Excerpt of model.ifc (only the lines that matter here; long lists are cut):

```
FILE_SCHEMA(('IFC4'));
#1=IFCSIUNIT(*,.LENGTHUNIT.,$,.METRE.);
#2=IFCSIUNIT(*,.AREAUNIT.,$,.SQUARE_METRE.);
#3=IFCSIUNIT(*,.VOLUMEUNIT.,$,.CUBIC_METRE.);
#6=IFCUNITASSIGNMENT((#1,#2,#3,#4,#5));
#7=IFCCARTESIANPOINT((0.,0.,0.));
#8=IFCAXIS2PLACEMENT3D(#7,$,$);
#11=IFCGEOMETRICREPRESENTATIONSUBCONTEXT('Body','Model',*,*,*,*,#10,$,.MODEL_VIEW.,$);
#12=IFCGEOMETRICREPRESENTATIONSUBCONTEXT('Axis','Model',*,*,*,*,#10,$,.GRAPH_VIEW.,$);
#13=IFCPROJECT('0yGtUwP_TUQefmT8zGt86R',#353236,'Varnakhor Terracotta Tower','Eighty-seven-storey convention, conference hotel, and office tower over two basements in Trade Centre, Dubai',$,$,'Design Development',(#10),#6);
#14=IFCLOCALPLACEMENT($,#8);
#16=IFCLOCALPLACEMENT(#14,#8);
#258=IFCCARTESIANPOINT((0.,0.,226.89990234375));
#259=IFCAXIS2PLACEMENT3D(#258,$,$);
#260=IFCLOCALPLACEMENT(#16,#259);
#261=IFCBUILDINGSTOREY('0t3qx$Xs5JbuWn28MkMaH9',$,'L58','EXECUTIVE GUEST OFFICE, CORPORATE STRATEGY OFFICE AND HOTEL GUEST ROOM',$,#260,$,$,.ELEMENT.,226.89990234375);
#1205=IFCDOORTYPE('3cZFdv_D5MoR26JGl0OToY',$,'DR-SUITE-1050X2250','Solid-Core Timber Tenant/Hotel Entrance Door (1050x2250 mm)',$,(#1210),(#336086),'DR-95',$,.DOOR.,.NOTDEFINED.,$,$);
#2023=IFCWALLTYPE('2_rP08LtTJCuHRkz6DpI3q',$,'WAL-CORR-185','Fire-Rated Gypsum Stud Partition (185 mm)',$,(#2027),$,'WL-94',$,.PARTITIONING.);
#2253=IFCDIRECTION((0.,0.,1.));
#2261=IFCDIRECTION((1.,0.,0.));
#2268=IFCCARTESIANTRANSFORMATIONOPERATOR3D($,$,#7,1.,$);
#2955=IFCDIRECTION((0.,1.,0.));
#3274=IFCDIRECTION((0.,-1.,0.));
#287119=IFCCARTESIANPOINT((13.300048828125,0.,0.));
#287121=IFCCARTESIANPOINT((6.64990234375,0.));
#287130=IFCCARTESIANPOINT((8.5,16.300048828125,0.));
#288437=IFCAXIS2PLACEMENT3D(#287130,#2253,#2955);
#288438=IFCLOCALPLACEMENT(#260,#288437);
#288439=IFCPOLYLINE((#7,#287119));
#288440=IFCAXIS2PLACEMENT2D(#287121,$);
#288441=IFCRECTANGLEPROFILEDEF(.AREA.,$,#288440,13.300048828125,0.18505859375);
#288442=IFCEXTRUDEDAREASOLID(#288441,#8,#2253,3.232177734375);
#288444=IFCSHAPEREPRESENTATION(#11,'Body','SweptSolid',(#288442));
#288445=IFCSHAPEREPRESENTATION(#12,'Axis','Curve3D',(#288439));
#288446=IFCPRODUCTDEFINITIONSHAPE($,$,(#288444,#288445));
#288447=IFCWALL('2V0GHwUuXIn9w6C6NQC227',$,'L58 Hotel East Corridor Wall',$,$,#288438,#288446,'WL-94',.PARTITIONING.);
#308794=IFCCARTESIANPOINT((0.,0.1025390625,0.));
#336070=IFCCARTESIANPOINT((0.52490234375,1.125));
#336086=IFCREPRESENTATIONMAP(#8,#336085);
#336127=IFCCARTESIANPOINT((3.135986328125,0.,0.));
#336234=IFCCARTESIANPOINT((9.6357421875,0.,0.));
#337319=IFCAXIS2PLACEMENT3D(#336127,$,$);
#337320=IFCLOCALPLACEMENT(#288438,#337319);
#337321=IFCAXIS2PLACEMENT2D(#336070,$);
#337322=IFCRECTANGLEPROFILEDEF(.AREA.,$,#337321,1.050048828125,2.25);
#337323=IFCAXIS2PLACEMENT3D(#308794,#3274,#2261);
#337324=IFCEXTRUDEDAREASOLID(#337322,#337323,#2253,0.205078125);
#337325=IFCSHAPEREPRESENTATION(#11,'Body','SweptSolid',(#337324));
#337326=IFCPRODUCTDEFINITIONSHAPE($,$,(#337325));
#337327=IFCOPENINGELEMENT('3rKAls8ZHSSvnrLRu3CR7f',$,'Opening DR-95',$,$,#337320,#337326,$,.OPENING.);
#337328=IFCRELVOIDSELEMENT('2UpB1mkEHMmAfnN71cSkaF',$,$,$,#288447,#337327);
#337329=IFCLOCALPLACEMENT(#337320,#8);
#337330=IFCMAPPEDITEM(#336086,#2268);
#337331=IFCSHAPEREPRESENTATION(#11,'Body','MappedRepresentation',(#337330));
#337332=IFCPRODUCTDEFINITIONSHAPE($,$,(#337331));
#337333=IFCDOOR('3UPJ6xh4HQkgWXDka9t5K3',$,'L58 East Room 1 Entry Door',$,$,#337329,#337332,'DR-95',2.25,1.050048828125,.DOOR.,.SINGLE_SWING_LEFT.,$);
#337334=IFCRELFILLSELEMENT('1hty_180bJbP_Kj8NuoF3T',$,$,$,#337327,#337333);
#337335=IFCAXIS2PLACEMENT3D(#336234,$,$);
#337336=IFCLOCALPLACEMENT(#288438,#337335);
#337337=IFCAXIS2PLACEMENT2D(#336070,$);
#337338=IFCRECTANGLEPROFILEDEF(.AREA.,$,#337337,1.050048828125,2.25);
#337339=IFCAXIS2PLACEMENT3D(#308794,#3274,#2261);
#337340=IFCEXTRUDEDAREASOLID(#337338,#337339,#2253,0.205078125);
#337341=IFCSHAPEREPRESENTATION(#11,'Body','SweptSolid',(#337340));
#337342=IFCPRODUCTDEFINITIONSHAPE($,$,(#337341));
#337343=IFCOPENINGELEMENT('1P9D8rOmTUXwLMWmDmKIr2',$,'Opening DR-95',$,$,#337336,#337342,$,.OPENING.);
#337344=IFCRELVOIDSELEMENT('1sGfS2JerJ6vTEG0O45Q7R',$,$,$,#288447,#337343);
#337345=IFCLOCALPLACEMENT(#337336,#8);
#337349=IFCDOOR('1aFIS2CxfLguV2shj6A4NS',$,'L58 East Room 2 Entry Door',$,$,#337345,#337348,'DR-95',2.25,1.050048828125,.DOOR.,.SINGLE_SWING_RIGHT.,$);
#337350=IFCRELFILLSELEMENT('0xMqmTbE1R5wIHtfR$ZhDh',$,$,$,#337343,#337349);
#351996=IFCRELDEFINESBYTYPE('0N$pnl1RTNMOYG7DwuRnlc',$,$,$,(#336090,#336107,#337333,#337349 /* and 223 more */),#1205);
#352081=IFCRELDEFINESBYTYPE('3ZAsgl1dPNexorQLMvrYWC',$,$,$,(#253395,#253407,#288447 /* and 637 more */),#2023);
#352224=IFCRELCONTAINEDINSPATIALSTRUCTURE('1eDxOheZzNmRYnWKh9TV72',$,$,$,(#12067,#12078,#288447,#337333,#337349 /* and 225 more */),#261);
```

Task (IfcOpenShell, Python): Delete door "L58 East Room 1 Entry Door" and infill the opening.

```python
import ifcopenshell
import ifcopenshell.api.feature
import ifcopenshell.api.root
import ifcopenshell.geom
import ifcopenshell.util.shape

model = ifcopenshell.open("model.ifc")
settings = ifcopenshell.geom.settings()


def volume(element):
    """Net volume in cubic metres, openings subtracted."""
    shape = ifcopenshell.geom.create_shape(settings, element)
    return ifcopenshell.util.shape.get_volume(shape.geometry)


door = model.by_id(337333)
opening = door.FillsVoids[0].RelatingOpeningElement
wall = opening.VoidsElements[0].RelatingBuildingElement
before = volume(wall)

ifcopenshell.api.root.remove_product(model, product=door)
ifcopenshell.api.feature.remove_feature(model, feature=opening)

after = volume(wall)

print(f"wall volume {before:.3f} -> {after:.3f} m3")

model.write("model_rev.ifc")
```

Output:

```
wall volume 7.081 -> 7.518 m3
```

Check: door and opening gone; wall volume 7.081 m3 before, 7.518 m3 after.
